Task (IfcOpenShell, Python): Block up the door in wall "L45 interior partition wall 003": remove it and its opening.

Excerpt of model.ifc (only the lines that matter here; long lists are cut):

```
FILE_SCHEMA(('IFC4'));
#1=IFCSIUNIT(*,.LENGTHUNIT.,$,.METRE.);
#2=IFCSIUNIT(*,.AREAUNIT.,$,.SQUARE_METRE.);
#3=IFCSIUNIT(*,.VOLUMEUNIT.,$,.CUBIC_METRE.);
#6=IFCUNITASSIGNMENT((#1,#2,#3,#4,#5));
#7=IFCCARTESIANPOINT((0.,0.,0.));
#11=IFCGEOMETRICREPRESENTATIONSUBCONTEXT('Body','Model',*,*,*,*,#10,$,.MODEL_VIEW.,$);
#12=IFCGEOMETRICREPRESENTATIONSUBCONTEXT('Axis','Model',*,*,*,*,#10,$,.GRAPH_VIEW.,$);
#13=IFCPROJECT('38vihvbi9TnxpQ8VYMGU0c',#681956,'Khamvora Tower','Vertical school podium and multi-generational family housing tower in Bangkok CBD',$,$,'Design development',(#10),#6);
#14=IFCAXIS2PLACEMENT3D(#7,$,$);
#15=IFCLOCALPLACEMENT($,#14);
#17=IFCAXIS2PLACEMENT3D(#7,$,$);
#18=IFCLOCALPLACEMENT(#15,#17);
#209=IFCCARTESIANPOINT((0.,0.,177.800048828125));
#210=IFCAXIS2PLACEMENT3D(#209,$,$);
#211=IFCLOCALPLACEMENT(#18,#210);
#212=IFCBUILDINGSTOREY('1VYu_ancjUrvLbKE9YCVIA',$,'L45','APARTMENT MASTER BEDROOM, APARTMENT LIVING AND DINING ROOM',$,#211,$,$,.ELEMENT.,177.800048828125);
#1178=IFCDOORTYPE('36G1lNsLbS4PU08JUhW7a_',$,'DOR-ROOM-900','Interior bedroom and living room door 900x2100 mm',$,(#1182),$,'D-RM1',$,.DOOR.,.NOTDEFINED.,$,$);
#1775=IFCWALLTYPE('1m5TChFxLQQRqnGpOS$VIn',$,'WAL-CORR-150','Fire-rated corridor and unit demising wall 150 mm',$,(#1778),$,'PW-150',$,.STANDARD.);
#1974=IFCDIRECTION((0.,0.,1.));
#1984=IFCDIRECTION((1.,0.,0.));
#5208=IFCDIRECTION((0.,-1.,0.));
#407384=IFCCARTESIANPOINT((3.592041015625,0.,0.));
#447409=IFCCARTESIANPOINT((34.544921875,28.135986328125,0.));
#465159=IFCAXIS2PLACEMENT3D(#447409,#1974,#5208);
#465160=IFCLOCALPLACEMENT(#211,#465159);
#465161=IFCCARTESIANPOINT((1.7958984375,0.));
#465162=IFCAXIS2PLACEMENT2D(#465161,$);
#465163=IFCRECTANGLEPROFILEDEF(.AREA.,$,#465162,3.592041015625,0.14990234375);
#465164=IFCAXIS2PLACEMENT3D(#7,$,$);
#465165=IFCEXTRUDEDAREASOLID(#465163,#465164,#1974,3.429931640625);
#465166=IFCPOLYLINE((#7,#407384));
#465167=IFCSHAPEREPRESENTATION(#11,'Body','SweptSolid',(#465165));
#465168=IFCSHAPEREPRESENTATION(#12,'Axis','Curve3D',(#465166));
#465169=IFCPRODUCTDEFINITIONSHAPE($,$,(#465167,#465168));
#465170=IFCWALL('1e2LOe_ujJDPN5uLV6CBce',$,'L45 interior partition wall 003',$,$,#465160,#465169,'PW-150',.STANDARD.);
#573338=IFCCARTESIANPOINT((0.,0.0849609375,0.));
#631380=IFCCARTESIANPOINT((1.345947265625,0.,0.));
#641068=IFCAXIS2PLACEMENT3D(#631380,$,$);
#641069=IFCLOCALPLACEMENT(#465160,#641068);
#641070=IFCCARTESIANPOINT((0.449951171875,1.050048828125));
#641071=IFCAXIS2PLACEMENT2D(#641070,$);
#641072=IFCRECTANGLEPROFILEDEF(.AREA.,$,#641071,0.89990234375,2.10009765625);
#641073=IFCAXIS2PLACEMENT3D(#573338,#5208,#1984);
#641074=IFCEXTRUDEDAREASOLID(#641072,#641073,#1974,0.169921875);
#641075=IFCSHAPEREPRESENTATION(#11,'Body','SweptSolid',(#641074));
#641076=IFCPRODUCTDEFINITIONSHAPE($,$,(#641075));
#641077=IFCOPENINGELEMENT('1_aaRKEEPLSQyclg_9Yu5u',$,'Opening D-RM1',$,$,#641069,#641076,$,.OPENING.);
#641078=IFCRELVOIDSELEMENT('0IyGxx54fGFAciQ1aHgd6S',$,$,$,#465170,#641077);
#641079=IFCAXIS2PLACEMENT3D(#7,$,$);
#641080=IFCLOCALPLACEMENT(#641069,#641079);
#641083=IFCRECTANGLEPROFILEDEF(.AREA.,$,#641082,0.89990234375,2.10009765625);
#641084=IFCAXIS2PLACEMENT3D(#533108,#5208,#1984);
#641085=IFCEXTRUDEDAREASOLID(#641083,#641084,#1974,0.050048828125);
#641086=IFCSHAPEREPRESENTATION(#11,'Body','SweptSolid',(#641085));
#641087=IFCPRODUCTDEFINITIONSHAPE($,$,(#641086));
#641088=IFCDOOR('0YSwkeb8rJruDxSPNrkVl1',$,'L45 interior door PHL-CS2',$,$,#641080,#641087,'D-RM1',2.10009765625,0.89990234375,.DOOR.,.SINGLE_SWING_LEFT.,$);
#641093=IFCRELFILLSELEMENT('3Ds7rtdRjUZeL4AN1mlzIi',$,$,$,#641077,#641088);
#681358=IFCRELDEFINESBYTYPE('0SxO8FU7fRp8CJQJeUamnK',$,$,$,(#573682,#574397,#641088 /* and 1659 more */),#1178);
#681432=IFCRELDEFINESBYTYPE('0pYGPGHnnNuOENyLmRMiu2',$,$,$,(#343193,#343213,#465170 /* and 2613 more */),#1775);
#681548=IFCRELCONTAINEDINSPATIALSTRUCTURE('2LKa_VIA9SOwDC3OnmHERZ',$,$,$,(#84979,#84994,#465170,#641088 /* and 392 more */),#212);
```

```python
import ifcopenshell
import ifcopenshell.api.feature
import ifcopenshell.api.root
import ifcopenshell.geom
import ifcopenshell.util.shape

model = ifcopenshell.open("model.ifc")
settings = ifcopenshell.geom.settings()


def volume(element):
    """Net volume in cubic metres, openings subtracted."""
    shape = ifcopenshell.geom.create_shape(settings, element)
    return ifcopenshell.util.shape.get_volume(shape.geometry)


door = model.by_guid("0YSwkeb8rJruDxSPNrkVl1")
opening = door.FillsVoids[0].RelatingOpeningElement
wall = opening.VoidsElements[0].RelatingBuildingElement
before = volume(wall)

ifcopenshell.api.root.remove_product(model, product=door)
ifcopenshell.api.feature.remove_feature(model, feature=opening)

after = volume(wall)

print(f"wall volume {before:.3f} -> {after:.3f} m3")

model.write("model_v2.ifc")
```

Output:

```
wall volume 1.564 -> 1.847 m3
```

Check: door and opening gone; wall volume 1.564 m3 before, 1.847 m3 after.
